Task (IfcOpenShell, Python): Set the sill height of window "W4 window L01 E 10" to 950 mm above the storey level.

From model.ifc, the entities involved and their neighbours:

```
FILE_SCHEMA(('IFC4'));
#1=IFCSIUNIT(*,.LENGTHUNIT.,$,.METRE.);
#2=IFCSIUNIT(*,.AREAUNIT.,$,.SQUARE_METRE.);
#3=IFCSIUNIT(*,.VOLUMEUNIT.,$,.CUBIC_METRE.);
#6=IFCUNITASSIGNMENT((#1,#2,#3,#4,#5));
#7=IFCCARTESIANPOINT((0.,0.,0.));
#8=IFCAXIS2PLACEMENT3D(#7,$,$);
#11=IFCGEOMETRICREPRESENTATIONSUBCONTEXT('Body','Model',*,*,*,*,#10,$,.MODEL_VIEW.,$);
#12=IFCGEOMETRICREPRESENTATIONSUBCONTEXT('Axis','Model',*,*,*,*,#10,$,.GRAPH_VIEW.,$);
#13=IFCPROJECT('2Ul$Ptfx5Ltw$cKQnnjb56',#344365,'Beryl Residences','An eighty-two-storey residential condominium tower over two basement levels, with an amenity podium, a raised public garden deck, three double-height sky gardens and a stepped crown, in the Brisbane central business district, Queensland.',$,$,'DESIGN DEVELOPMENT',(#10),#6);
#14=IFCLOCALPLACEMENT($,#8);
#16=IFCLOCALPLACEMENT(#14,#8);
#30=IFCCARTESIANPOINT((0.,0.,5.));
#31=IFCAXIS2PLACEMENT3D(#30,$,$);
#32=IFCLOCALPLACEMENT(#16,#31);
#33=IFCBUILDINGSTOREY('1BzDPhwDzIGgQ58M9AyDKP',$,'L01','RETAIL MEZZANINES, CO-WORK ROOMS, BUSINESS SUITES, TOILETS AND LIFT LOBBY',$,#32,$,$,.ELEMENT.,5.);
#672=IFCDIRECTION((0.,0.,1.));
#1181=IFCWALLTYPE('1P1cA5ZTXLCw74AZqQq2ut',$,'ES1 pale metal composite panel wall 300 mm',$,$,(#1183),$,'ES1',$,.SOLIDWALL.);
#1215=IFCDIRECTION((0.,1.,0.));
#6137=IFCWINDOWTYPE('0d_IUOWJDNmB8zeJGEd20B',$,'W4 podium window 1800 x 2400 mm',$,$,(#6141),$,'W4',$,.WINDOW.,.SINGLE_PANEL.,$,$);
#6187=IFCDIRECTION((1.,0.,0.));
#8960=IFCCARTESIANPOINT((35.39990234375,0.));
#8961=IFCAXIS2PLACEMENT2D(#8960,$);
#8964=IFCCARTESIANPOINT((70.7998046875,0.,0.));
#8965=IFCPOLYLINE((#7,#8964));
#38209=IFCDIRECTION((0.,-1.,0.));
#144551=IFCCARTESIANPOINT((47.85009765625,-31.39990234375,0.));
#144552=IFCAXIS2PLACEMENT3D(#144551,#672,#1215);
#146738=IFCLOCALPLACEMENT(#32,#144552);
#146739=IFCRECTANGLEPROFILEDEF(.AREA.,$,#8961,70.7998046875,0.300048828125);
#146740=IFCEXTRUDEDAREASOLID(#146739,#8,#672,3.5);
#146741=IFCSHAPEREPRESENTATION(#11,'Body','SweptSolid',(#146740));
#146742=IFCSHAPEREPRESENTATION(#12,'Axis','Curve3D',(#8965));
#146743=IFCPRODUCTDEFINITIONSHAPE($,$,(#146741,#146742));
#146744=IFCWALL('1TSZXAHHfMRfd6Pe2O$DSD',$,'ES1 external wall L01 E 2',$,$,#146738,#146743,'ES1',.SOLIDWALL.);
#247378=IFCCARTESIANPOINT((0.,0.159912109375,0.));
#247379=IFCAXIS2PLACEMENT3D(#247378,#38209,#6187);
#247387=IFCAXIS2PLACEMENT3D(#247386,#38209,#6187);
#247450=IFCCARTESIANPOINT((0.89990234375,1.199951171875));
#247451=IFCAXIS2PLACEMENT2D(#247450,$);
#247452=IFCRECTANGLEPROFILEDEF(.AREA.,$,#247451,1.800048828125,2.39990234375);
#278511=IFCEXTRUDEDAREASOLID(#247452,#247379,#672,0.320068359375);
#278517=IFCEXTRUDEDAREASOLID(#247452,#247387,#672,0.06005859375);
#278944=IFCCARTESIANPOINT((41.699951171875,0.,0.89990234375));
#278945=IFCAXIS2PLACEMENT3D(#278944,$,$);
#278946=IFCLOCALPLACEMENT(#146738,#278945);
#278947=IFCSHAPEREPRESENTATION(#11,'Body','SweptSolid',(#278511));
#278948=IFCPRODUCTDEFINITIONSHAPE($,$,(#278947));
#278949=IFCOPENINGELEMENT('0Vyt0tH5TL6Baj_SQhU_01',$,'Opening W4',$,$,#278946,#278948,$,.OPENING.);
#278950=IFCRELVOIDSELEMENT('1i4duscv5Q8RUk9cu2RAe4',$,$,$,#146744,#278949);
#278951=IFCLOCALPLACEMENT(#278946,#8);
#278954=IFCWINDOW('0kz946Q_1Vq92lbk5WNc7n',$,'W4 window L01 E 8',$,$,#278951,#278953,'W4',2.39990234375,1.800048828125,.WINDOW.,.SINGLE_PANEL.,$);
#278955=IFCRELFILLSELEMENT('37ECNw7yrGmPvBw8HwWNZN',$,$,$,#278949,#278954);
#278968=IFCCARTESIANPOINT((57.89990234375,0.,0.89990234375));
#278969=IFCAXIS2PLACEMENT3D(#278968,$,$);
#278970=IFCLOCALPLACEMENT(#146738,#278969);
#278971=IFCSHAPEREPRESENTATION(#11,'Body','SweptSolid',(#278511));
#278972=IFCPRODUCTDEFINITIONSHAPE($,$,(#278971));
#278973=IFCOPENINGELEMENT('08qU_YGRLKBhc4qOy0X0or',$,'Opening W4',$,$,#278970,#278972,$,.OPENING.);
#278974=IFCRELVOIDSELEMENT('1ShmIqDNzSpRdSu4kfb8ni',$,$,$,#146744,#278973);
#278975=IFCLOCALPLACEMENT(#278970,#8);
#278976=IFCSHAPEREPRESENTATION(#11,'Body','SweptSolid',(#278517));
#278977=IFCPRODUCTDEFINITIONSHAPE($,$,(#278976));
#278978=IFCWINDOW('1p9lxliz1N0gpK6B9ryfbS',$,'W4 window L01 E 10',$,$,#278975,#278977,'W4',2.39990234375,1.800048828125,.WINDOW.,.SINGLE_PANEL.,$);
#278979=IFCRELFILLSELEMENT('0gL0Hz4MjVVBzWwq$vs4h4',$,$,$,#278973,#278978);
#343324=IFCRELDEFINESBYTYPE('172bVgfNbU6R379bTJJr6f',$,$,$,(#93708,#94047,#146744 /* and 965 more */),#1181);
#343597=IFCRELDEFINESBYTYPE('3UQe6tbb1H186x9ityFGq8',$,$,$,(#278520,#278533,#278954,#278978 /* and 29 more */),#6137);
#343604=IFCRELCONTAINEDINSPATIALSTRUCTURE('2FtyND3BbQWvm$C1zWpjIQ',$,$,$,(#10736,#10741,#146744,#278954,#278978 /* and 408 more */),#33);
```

```python
import numpy as np
import ifcopenshell
import ifcopenshell.api.geometry
import ifcopenshell.geom
import ifcopenshell.util.element
import ifcopenshell.util.placement
import ifcopenshell.util.shape
import ifcopenshell.util.unit

model = ifcopenshell.open("model.ifc")
unit_scale = ifcopenshell.util.unit.calculate_unit_scale(model)

window = model.by_guid("1p9lxliz1N0gpK6B9ryfbS")
opening = window.FillsVoids[0].RelatingOpeningElement
storey = ifcopenshell.util.element.get_container(window, ifc_class="IfcBuildingStorey")
level = ifcopenshell.util.placement.get_local_placement(storey.ObjectPlacement)[2, 3]

# The opening's origin need not be at the sill, so measure its lowest point.
shape = ifcopenshell.geom.create_shape(ifcopenshell.geom.settings(), opening)
bottom = ifcopenshell.util.shape.get_shape_bottom_elevation(shape, shape.geometry) / unit_scale
dz = level + 0.95 / unit_scale - bottom

shift = np.array([0.0, 0.0, dz])
# The window is placed relative to its opening, so it follows when the opening moves.
matrix = ifcopenshell.util.placement.get_local_placement(opening.ObjectPlacement)
matrix[:3, 3] += shift
ifcopenshell.api.geometry.edit_object_placement(
    model, product=opening, matrix=matrix, is_si=False, should_transform_children=True
)

print(f"moved by {dz * unit_scale:+.3f} m")

model.write("model-out.ifc")
```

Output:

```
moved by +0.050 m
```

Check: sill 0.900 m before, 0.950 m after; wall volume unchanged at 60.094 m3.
